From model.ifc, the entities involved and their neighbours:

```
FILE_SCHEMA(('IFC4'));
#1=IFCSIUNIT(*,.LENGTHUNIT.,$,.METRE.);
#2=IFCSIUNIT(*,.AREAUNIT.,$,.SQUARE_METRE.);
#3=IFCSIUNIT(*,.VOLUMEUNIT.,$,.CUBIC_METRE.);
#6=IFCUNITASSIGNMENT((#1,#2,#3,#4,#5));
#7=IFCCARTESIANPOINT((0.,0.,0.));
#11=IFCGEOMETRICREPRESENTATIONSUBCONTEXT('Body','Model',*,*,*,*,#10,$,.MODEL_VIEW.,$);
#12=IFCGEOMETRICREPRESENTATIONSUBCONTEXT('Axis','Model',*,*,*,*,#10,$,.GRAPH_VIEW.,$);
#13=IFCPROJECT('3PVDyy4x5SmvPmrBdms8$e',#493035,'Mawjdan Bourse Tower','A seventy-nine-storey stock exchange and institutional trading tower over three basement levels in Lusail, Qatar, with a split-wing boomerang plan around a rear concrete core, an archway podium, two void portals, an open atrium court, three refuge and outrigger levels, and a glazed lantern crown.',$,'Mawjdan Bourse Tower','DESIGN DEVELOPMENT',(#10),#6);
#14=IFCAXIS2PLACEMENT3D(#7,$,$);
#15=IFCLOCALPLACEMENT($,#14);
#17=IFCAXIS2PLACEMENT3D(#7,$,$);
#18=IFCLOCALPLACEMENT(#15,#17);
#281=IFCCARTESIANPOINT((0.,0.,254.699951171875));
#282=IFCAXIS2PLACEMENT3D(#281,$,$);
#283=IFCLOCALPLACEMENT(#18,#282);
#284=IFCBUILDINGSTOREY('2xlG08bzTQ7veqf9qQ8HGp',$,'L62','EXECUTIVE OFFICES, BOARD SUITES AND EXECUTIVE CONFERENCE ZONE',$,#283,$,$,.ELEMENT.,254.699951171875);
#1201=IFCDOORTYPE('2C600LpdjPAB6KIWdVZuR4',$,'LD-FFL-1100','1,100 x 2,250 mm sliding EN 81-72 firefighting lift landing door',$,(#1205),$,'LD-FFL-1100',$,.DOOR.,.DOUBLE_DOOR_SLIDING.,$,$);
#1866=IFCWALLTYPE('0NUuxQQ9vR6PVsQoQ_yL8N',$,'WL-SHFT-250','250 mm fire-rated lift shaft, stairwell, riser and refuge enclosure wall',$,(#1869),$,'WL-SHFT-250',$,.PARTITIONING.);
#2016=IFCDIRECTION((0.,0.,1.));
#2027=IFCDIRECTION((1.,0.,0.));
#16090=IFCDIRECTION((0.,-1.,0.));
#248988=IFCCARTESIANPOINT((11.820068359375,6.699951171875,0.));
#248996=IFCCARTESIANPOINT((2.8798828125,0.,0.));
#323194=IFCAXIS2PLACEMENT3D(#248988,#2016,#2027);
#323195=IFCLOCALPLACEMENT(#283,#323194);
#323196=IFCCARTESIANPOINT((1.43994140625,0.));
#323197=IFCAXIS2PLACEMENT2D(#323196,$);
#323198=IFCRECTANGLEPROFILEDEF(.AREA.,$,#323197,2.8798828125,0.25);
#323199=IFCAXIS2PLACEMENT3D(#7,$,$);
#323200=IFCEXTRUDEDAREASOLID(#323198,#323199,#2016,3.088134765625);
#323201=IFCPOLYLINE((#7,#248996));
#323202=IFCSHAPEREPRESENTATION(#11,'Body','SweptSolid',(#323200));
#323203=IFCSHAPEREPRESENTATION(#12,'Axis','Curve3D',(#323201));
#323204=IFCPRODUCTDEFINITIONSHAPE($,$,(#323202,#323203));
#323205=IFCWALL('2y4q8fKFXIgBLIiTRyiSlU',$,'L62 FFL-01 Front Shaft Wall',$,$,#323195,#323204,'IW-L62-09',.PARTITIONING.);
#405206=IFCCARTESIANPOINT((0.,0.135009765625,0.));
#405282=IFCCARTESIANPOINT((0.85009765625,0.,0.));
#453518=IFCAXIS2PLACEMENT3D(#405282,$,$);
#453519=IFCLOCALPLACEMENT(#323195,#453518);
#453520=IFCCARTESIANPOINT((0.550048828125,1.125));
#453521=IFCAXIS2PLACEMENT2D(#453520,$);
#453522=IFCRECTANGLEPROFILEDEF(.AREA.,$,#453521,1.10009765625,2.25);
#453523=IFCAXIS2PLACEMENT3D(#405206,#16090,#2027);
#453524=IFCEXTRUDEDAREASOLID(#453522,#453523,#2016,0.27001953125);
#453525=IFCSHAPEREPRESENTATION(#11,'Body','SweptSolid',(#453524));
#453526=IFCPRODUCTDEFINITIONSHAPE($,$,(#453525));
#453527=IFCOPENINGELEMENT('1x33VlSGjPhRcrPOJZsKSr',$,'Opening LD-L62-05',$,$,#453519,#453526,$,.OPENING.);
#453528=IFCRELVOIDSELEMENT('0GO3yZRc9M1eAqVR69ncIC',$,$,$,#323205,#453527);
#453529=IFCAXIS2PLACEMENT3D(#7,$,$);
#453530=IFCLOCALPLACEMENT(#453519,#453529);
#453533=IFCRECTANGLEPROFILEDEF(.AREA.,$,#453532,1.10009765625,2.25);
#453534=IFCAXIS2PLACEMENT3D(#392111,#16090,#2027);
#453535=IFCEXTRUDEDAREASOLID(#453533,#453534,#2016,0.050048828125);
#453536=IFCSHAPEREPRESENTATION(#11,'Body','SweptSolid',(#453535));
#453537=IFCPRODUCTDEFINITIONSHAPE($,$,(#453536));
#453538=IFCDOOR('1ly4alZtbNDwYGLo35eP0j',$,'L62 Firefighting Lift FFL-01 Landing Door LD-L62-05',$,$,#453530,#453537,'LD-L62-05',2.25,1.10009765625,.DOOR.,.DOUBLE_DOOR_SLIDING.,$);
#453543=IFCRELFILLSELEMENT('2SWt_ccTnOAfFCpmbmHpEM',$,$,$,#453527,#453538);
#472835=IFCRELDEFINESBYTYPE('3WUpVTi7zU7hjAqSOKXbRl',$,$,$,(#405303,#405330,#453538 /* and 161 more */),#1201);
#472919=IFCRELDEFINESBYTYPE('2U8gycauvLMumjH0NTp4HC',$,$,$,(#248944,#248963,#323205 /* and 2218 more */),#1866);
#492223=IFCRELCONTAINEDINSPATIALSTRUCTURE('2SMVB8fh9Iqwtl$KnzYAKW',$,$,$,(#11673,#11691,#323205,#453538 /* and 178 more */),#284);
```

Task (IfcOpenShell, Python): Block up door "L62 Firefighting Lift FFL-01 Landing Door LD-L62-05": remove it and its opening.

```python
import ifcopenshell
import ifcopenshell.api.feature
import ifcopenshell.api.root
import ifcopenshell.geom
import ifcopenshell.util.shape

model = ifcopenshell.open("model.ifc")
settings = ifcopenshell.geom.settings()


def volume(element):
    """Net volume in cubic metres, openings subtracted."""
    shape = ifcopenshell.geom.create_shape(settings, element)
    return ifcopenshell.util.shape.get_volume(shape.geometry)


door = model.by_guid("1ly4alZtbNDwYGLo35eP0j")
opening = door.FillsVoids[0].RelatingOpeningElement
wall = opening.VoidsElements[0].RelatingBuildingElement
before = volume(wall)

ifcopenshell.api.root.remove_product(model, product=door)
ifcopenshell.api.feature.remove_feature(model, feature=opening)

after = volume(wall)

print(f"wall volume {before:.3f} -> {after:.3f} m3")

model.write("model_rev.ifc")
```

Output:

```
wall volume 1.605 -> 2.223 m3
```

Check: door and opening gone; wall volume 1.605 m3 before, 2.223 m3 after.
